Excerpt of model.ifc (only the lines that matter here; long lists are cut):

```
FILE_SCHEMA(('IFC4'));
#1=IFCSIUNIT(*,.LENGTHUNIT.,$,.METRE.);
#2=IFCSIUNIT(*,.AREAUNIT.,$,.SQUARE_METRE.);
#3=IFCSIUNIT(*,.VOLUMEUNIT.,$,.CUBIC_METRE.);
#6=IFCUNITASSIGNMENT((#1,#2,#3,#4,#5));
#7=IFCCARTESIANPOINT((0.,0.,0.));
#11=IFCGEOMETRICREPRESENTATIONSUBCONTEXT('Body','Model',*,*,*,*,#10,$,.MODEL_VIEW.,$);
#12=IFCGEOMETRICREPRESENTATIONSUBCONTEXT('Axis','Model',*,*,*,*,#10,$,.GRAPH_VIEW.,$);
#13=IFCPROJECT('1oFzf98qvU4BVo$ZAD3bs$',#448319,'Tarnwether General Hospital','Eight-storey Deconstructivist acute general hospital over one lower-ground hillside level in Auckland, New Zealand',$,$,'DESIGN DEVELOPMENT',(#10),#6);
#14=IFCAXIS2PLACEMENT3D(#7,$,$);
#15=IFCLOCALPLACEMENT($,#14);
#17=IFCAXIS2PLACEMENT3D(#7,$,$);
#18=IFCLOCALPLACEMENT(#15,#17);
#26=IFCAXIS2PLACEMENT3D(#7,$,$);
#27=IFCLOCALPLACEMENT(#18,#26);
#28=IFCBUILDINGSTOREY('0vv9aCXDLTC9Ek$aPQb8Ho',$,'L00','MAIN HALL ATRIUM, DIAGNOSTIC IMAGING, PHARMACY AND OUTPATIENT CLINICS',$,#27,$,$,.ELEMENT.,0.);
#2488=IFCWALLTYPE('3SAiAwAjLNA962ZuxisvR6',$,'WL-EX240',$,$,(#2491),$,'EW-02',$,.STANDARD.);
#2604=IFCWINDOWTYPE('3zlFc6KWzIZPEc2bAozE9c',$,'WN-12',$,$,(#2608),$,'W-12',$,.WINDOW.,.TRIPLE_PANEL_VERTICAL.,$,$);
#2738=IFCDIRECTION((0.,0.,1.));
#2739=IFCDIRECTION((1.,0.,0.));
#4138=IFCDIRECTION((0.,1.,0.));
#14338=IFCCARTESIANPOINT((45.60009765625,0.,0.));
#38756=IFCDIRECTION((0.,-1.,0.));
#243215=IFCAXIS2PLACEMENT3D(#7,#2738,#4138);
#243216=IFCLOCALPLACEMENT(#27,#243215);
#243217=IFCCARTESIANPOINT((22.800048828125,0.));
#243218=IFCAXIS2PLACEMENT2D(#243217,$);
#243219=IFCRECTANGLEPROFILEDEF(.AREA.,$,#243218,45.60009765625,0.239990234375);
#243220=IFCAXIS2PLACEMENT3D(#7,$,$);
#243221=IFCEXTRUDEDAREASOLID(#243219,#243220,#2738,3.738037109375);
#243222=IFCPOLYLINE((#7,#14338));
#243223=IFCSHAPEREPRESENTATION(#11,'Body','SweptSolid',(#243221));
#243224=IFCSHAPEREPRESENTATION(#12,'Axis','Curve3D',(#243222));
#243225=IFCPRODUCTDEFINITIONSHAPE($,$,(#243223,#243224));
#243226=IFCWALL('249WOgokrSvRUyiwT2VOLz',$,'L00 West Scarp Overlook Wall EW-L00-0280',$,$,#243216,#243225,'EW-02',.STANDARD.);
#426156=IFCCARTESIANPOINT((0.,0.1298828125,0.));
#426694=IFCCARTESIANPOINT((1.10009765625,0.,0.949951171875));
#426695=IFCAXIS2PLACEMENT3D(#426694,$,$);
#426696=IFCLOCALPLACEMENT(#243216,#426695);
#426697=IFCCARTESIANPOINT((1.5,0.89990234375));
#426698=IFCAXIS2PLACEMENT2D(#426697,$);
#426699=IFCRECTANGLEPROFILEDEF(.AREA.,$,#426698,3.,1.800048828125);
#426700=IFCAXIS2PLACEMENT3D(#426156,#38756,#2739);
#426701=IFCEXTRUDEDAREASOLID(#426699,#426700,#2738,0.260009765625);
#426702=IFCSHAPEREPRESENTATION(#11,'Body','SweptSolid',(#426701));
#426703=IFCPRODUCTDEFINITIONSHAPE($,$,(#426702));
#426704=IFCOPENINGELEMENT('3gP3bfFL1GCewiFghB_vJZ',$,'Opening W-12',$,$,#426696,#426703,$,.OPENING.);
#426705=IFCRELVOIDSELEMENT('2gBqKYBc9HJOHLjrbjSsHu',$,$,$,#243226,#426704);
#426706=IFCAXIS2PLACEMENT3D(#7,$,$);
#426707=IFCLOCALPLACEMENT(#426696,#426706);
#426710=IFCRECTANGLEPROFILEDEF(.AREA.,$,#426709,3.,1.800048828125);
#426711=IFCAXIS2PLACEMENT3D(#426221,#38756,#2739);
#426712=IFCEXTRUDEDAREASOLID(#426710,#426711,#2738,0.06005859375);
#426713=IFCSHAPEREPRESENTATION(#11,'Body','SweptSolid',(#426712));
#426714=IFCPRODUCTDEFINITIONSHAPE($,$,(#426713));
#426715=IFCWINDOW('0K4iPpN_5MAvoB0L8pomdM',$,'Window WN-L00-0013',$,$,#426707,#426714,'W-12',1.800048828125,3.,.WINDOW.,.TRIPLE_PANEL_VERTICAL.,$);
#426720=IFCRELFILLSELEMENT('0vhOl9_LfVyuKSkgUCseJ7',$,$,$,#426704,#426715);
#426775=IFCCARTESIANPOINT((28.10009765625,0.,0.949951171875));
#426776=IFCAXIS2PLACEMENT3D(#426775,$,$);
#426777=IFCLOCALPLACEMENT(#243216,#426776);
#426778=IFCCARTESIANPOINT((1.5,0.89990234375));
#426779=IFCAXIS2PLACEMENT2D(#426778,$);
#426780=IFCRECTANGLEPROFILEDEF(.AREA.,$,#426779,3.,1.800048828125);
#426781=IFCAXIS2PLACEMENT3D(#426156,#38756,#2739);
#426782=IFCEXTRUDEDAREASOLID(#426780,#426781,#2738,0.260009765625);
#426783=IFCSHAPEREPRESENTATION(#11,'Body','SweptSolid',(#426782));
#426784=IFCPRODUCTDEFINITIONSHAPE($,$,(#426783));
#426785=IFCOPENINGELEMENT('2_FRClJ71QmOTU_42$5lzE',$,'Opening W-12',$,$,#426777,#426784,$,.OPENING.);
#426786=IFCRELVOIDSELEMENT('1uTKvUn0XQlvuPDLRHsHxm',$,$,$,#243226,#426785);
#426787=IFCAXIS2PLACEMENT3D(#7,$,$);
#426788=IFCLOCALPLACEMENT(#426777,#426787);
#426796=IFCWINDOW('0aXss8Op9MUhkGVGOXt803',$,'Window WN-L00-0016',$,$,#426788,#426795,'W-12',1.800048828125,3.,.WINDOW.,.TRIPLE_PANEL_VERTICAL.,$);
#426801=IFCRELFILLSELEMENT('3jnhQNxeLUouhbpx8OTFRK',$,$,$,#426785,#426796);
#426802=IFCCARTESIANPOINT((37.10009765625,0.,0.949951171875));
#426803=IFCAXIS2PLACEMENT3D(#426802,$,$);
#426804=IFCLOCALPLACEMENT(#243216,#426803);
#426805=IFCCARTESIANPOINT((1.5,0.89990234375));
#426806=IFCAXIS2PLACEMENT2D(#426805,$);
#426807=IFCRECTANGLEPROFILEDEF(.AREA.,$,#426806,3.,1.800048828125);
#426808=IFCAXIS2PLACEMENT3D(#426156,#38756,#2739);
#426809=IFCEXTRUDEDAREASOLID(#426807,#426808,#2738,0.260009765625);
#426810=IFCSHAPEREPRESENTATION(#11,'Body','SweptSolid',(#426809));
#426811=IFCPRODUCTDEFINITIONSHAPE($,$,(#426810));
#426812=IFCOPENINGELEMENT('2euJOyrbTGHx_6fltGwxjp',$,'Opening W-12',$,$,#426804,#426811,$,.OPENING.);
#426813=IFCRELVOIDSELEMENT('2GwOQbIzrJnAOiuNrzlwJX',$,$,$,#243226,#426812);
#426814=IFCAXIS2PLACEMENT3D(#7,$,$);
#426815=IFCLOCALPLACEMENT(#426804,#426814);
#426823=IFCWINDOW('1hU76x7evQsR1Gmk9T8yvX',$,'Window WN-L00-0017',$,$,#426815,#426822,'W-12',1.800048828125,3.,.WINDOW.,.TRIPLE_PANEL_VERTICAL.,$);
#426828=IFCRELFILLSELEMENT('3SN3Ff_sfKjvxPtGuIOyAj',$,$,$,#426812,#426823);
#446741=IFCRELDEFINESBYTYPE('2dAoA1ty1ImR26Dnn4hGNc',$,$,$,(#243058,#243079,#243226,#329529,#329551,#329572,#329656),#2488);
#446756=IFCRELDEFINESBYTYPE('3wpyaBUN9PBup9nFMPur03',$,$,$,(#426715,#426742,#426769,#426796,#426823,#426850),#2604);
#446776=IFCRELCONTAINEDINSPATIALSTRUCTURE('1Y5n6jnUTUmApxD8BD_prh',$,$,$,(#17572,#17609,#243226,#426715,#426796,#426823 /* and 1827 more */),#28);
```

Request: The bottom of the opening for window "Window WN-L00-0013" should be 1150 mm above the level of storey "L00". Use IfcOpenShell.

```python
import numpy as np
import ifcopenshell
import ifcopenshell.api.geometry
import ifcopenshell.geom
import ifcopenshell.util.element
import ifcopenshell.util.placement
import ifcopenshell.util.shape
import ifcopenshell.util.unit

model = ifcopenshell.open("model.ifc")
unit_scale = ifcopenshell.util.unit.calculate_unit_scale(model)

window = model.by_guid("0K4iPpN_5MAvoB0L8pomdM")
opening = window.FillsVoids[0].RelatingOpeningElement
storey = ifcopenshell.util.element.get_container(window, ifc_class="IfcBuildingStorey")
level = ifcopenshell.util.placement.get_local_placement(storey.ObjectPlacement)[2, 3]

# The opening's origin need not be at the sill, so measure its lowest point.
shape = ifcopenshell.geom.create_shape(ifcopenshell.geom.settings(), opening)
bottom = ifcopenshell.util.shape.get_shape_bottom_elevation(shape, shape.geometry) / unit_scale
dz = level + 1.15 / unit_scale - bottom

shift = np.array([0.0, 0.0, dz])
# The window is placed relative to its opening, so it follows when the opening moves.
matrix = ifcopenshell.util.placement.get_local_placement(opening.ObjectPlacement)
matrix[:3, 3] += shift
ifcopenshell.api.geometry.edit_object_placement(
    model, product=opening, matrix=matrix, is_si=False, should_transform_children=True
)

print(f"moved by {dz * unit_scale:+.3f} m")

model.write("model_updated.ifc")
```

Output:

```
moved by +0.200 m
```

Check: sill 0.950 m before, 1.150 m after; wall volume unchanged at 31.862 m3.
